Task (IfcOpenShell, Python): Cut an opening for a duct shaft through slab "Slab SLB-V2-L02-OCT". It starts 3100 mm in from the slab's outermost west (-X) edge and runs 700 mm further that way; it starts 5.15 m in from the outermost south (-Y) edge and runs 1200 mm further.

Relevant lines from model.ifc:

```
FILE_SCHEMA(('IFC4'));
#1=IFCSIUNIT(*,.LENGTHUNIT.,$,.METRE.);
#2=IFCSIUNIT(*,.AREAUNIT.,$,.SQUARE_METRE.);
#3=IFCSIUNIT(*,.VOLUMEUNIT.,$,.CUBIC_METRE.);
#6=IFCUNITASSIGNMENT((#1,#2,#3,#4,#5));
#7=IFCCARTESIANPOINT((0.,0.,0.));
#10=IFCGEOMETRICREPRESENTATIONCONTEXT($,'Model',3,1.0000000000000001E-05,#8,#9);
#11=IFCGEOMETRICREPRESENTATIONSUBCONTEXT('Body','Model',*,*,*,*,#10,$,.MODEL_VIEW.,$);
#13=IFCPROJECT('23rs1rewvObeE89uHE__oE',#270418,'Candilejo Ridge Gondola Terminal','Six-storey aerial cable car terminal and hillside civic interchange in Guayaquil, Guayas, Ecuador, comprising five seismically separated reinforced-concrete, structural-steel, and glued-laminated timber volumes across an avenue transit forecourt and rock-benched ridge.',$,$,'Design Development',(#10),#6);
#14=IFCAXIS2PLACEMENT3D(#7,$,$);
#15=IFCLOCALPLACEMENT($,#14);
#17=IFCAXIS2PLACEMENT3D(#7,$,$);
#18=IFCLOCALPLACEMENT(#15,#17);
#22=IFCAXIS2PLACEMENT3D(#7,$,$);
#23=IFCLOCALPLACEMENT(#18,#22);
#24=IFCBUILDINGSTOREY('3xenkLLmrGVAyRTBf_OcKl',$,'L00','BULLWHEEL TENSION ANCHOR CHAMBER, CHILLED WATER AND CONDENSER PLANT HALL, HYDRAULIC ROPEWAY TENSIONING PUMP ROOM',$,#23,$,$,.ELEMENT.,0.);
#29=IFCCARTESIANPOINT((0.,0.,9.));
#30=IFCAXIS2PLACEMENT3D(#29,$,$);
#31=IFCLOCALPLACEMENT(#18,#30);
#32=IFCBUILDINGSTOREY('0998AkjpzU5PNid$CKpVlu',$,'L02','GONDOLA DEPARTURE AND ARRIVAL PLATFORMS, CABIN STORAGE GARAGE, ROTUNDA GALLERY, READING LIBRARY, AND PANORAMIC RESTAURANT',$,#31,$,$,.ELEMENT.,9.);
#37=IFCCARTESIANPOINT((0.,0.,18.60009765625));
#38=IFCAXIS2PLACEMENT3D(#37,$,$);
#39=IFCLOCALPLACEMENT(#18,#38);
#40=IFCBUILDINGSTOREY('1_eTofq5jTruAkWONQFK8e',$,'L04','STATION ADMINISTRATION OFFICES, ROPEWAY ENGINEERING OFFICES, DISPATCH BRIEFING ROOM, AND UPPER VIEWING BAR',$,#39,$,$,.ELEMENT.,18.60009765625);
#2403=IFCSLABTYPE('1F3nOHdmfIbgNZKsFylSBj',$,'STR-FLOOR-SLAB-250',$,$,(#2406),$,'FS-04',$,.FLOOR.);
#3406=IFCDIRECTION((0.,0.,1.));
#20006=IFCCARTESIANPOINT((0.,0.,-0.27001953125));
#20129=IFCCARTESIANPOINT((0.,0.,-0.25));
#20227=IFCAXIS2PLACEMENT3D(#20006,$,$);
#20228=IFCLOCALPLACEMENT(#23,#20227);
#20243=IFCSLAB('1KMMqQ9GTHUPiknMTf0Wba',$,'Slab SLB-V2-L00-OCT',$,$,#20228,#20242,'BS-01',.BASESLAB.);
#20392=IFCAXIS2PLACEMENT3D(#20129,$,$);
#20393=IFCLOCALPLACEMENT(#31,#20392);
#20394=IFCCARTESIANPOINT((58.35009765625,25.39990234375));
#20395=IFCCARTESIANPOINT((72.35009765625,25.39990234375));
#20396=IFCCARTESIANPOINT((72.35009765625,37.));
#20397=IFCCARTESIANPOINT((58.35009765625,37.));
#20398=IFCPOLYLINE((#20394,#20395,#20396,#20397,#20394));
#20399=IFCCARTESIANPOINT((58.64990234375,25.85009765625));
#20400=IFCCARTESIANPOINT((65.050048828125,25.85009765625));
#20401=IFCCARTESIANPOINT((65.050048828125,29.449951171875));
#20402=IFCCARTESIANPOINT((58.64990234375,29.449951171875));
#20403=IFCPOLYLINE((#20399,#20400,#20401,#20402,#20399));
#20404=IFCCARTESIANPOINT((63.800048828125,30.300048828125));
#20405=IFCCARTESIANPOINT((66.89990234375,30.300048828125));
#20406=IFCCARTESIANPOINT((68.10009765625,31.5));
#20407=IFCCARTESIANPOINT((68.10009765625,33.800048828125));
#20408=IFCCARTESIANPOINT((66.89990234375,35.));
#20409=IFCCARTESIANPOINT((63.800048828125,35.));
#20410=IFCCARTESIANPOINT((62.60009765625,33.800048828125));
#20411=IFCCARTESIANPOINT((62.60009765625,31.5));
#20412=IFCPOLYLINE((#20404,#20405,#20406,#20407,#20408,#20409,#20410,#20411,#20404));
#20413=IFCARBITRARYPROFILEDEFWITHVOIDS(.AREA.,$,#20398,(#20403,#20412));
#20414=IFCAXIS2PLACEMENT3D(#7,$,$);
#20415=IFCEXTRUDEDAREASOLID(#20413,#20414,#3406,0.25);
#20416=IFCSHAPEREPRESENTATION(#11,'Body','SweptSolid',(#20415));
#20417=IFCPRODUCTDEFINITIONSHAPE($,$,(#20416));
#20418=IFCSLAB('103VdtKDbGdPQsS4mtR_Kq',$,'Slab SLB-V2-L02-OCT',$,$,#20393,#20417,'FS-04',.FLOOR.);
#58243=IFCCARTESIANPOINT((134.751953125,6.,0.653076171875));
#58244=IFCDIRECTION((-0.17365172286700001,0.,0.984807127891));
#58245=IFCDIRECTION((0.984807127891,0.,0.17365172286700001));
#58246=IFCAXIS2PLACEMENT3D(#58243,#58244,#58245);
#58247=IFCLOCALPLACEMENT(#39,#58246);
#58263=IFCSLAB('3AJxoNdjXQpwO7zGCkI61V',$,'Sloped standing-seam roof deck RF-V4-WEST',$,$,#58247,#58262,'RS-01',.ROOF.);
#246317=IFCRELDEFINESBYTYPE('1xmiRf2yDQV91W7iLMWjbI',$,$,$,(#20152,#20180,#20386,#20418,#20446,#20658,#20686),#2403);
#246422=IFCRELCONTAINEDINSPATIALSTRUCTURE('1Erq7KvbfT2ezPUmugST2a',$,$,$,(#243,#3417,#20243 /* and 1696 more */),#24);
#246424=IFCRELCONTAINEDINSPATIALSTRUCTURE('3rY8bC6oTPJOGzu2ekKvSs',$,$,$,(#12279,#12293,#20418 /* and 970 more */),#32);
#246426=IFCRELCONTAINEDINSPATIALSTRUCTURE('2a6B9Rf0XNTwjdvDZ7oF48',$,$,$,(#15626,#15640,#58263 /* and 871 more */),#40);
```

```python
import numpy as np
import ifcopenshell
import ifcopenshell.api.feature
import ifcopenshell.api.geometry
import ifcopenshell.api.root
import ifcopenshell.geom
import ifcopenshell.util.placement
import ifcopenshell.util.representation
import ifcopenshell.util.shape
import ifcopenshell.util.unit

model = ifcopenshell.open("model.ifc")
unit_scale = ifcopenshell.util.unit.calculate_unit_scale(model)
settings = ifcopenshell.geom.settings()


def volume(element):
    """Net volume in cubic metres, openings subtracted."""
    shape = ifcopenshell.geom.create_shape(settings, element)
    return ifcopenshell.util.shape.get_volume(shape.geometry)


slab = model.by_id(20418)
before = volume(slab)

# Extent in the slab's own axes, in metres. The edges named are its -X and -Y sides.
slab_shape = ifcopenshell.geom.create_shape(settings, slab)
vertices = ifcopenshell.util.shape.get_vertices(slab_shape.geometry)
x_min, y_min, bottom = vertices.min(axis=0)
top = vertices[:, 2].max()

opening = ifcopenshell.api.root.create_entity(model, ifc_class="IfcOpeningElement", name="Duct shaft opening", predefined_type="OPENING")
context = ifcopenshell.util.representation.get_context(model, "Model", "Body", "MODEL_VIEW")
width, depth = 0.7, 1.2
outline = [(0.0, 0.0), (width, 0.0), (width, depth), (0.0, depth), (0.0, 0.0)]
# Overshoot both faces by 50 mm so the cut is clean.
shape = ifcopenshell.api.geometry.add_slab_representation(
    model, context=context, depth=top - bottom + 0.1, polyline=outline
)
ifcopenshell.api.geometry.assign_representation(model, product=opening, representation=shape)

matrix = ifcopenshell.util.placement.get_local_placement(slab.ObjectPlacement)
matrix[:, 3] = matrix @ np.append(np.array([x_min + 3.1, y_min + 5.15, bottom - 0.05]) / unit_scale, 1.0)
ifcopenshell.api.geometry.edit_object_placement(model, product=opening, matrix=matrix, is_si=False)
ifcopenshell.api.feature.add_feature(model, feature=opening, element=slab)

after = volume(slab)

print(f"slab volume {before:.3f} -> {after:.3f} m3")

model.write("model_edited.ifc")
```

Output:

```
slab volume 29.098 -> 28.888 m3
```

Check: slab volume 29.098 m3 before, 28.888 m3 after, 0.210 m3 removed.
